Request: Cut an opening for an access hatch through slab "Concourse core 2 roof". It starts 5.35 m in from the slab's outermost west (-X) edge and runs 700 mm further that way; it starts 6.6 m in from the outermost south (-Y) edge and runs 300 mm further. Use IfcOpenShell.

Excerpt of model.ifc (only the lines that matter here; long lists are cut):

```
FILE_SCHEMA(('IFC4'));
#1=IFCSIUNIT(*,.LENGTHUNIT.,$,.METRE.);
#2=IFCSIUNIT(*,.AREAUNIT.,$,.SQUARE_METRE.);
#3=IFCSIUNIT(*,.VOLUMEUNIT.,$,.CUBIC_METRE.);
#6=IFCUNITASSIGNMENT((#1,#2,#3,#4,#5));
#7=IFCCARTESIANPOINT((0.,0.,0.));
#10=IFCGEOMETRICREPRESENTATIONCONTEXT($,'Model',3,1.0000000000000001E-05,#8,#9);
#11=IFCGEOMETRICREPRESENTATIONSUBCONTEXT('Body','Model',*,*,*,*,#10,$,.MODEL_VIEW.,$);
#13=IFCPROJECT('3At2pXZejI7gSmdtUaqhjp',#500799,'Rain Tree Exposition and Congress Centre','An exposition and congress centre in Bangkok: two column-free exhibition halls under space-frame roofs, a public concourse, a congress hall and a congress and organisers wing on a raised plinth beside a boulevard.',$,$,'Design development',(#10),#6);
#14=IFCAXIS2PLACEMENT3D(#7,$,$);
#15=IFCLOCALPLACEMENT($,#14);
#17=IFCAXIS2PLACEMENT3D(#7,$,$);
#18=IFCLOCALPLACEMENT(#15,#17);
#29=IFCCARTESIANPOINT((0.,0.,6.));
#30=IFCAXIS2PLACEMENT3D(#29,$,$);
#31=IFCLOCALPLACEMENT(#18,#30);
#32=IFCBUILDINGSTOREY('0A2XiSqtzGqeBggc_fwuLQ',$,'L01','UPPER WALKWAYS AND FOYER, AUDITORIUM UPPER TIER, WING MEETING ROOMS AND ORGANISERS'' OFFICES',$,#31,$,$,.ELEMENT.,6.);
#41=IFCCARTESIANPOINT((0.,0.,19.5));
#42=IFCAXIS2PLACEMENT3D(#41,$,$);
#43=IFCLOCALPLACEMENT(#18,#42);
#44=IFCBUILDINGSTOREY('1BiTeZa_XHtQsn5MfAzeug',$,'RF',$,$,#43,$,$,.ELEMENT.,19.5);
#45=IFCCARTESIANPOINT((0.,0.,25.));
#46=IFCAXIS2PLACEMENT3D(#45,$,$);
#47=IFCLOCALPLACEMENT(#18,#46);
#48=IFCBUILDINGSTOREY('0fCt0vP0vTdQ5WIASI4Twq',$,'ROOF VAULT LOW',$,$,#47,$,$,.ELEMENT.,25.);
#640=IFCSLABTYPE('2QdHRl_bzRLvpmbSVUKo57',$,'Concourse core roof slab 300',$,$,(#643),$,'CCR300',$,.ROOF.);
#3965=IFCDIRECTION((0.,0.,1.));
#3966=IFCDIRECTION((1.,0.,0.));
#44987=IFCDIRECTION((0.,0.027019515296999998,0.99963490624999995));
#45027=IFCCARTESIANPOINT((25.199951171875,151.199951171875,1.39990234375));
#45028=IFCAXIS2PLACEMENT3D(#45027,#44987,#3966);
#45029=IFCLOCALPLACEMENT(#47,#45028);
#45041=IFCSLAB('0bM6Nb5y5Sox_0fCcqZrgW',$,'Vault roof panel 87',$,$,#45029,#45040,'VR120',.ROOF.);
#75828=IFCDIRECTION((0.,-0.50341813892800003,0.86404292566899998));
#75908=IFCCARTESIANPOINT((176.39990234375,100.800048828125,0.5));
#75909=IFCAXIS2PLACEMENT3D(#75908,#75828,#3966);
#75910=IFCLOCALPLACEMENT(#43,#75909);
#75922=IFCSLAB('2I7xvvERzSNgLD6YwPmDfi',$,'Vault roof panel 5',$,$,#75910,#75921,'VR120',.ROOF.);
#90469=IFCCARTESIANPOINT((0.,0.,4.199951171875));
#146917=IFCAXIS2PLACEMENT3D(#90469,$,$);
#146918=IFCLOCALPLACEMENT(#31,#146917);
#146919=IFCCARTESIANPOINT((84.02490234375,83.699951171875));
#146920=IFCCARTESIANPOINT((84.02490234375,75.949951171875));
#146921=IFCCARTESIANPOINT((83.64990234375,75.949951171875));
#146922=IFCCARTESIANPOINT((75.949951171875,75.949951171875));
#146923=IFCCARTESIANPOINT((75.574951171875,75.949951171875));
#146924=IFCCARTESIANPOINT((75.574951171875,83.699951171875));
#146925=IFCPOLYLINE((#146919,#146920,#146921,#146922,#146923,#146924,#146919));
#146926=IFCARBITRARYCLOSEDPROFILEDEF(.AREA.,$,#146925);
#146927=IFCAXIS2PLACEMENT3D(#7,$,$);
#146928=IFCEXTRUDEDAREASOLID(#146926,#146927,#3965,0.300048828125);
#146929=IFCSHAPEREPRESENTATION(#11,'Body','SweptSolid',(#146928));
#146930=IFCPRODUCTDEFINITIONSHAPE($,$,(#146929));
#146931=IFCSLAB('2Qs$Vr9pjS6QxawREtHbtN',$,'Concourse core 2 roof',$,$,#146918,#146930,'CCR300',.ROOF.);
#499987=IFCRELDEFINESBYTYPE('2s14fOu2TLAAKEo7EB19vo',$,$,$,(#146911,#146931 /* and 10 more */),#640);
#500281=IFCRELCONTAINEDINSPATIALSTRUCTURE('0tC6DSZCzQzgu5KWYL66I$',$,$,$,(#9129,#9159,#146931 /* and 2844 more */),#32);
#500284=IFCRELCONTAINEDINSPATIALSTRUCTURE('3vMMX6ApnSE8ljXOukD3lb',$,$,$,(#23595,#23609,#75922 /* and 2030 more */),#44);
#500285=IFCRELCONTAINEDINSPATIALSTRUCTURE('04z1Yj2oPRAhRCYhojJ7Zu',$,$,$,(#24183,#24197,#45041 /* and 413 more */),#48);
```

```python
import numpy as np
import ifcopenshell
import ifcopenshell.api.feature
import ifcopenshell.api.geometry
import ifcopenshell.api.root
import ifcopenshell.geom
import ifcopenshell.util.placement
import ifcopenshell.util.representation
import ifcopenshell.util.shape
import ifcopenshell.util.unit

model = ifcopenshell.open("model.ifc")
unit_scale = ifcopenshell.util.unit.calculate_unit_scale(model)
settings = ifcopenshell.geom.settings()


def volume(element):
    """Net volume in cubic metres, openings subtracted."""
    shape = ifcopenshell.geom.create_shape(settings, element)
    return ifcopenshell.util.shape.get_volume(shape.geometry)


slab = model.by_id(146931)
before = volume(slab)

# Extent in the slab's own axes, in metres. The edges named are its -X and -Y sides.
slab_shape = ifcopenshell.geom.create_shape(settings, slab)
vertices = ifcopenshell.util.shape.get_vertices(slab_shape.geometry)
x_min, y_min, bottom = vertices.min(axis=0)
top = vertices[:, 2].max()

opening = ifcopenshell.api.root.create_entity(model, ifc_class="IfcOpeningElement", name="Access hatch opening", predefined_type="OPENING")
context = ifcopenshell.util.representation.get_context(model, "Model", "Body", "MODEL_VIEW")
width, depth = 0.7, 0.3
outline = [(0.0, 0.0), (width, 0.0), (width, depth), (0.0, depth), (0.0, 0.0)]
# Overshoot both faces by 50 mm so the cut is clean.
shape = ifcopenshell.api.geometry.add_slab_representation(
    model, context=context, depth=top - bottom + 0.1, polyline=outline
)
ifcopenshell.api.geometry.assign_representation(model, product=opening, representation=shape)

matrix = ifcopenshell.util.placement.get_local_placement(slab.ObjectPlacement)
matrix[:, 3] = matrix @ np.append(np.array([x_min + 5.35, y_min + 6.6, bottom - 0.05]) / unit_scale, 1.0)
ifcopenshell.api.geometry.edit_object_placement(model, product=opening, matrix=matrix, is_si=False)
ifcopenshell.api.feature.add_feature(model, feature=opening, element=slab)

after = volume(slab)

print(f"slab volume {before:.3f} -> {after:.3f} m3")

model.write("model_v2.ifc")
```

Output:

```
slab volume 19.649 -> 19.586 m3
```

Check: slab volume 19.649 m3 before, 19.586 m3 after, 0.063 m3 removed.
